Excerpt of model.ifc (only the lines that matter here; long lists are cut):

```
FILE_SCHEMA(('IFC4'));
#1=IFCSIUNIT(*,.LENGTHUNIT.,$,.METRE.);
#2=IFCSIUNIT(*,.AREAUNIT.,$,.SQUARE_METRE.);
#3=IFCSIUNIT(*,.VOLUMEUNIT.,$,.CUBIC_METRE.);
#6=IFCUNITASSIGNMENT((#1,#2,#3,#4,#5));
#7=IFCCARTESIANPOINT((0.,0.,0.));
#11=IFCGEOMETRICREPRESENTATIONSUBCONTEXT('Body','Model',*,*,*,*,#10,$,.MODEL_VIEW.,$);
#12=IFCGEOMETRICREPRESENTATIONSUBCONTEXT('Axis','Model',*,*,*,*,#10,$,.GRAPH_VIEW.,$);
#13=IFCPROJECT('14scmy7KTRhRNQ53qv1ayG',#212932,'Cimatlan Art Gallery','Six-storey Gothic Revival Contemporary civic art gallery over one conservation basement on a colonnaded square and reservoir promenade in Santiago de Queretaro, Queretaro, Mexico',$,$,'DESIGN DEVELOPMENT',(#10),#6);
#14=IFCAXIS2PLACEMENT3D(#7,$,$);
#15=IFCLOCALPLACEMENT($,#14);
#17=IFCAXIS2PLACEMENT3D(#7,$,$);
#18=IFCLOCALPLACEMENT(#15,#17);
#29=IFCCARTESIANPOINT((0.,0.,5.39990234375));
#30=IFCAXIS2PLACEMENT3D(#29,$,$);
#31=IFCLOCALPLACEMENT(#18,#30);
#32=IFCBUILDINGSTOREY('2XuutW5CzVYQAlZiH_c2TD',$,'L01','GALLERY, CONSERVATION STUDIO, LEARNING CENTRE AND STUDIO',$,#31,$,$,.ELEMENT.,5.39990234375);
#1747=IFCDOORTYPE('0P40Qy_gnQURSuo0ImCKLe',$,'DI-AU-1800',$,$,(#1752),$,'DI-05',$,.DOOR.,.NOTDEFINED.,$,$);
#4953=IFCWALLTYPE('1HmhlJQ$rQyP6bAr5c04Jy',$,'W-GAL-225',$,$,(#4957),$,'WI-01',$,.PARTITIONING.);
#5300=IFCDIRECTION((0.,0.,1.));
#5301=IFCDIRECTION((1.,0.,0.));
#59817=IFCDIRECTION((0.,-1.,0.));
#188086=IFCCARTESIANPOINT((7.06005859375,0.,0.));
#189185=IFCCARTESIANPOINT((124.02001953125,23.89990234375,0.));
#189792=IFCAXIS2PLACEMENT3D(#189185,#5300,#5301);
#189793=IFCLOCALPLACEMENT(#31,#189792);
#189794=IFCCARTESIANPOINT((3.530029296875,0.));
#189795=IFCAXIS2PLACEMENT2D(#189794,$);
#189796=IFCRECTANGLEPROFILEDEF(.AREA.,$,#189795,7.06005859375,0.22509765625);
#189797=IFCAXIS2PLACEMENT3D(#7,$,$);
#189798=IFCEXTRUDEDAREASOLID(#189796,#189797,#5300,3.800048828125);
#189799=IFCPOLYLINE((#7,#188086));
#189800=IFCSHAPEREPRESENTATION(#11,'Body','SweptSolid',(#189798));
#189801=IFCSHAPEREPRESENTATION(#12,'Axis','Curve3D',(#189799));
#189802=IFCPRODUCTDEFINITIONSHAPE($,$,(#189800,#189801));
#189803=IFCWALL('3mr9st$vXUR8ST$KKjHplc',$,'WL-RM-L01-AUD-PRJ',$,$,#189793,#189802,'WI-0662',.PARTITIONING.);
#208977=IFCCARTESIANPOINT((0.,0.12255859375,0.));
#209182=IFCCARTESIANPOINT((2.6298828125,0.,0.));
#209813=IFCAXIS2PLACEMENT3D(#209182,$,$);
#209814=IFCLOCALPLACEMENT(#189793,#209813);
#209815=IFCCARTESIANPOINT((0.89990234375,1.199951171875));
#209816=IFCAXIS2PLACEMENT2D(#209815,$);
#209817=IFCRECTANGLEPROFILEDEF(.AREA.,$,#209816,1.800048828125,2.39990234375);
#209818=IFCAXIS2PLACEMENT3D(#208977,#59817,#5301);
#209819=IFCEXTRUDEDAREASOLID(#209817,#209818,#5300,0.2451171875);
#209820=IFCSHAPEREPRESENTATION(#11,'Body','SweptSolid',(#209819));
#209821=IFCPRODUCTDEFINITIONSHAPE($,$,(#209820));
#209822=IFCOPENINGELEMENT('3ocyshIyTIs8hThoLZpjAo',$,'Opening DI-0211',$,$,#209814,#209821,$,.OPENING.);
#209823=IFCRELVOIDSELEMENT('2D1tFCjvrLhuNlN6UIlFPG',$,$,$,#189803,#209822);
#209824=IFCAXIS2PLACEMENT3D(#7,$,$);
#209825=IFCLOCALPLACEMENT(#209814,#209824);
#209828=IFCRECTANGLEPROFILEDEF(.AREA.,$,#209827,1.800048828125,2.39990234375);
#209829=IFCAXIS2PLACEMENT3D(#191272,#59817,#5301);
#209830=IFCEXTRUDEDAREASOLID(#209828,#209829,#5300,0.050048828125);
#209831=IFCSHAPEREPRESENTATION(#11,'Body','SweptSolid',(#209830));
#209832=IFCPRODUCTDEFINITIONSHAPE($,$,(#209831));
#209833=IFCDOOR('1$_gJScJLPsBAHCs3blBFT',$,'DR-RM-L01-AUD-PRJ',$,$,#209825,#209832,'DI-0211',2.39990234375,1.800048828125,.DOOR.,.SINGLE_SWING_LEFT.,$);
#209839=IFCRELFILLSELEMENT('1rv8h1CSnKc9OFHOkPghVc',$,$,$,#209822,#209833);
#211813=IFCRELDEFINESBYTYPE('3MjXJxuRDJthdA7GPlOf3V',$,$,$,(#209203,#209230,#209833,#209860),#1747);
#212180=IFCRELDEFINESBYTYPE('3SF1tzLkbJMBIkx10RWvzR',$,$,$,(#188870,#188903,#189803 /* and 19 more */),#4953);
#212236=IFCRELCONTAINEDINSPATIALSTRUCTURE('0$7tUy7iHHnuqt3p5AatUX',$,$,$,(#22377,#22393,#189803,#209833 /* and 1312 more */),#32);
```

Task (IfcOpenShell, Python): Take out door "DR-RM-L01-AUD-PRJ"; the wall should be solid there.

```python
import ifcopenshell
import ifcopenshell.api.feature
import ifcopenshell.api.root
import ifcopenshell.geom
import ifcopenshell.util.shape

model = ifcopenshell.open("model.ifc")
settings = ifcopenshell.geom.settings()


def volume(element):
    """Net volume in cubic metres, openings subtracted."""
    shape = ifcopenshell.geom.create_shape(settings, element)
    return ifcopenshell.util.shape.get_volume(shape.geometry)


door = model.by_id(209833)
opening = door.FillsVoids[0].RelatingOpeningElement
wall = opening.VoidsElements[0].RelatingBuildingElement
before = volume(wall)

ifcopenshell.api.root.remove_product(model, product=door)
ifcopenshell.api.feature.remove_feature(model, feature=opening)

after = volume(wall)

print(f"wall volume {before:.3f} -> {after:.3f} m3")

model.write("model-out.ifc")
```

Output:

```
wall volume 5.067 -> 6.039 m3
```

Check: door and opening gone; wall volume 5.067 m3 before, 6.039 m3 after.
